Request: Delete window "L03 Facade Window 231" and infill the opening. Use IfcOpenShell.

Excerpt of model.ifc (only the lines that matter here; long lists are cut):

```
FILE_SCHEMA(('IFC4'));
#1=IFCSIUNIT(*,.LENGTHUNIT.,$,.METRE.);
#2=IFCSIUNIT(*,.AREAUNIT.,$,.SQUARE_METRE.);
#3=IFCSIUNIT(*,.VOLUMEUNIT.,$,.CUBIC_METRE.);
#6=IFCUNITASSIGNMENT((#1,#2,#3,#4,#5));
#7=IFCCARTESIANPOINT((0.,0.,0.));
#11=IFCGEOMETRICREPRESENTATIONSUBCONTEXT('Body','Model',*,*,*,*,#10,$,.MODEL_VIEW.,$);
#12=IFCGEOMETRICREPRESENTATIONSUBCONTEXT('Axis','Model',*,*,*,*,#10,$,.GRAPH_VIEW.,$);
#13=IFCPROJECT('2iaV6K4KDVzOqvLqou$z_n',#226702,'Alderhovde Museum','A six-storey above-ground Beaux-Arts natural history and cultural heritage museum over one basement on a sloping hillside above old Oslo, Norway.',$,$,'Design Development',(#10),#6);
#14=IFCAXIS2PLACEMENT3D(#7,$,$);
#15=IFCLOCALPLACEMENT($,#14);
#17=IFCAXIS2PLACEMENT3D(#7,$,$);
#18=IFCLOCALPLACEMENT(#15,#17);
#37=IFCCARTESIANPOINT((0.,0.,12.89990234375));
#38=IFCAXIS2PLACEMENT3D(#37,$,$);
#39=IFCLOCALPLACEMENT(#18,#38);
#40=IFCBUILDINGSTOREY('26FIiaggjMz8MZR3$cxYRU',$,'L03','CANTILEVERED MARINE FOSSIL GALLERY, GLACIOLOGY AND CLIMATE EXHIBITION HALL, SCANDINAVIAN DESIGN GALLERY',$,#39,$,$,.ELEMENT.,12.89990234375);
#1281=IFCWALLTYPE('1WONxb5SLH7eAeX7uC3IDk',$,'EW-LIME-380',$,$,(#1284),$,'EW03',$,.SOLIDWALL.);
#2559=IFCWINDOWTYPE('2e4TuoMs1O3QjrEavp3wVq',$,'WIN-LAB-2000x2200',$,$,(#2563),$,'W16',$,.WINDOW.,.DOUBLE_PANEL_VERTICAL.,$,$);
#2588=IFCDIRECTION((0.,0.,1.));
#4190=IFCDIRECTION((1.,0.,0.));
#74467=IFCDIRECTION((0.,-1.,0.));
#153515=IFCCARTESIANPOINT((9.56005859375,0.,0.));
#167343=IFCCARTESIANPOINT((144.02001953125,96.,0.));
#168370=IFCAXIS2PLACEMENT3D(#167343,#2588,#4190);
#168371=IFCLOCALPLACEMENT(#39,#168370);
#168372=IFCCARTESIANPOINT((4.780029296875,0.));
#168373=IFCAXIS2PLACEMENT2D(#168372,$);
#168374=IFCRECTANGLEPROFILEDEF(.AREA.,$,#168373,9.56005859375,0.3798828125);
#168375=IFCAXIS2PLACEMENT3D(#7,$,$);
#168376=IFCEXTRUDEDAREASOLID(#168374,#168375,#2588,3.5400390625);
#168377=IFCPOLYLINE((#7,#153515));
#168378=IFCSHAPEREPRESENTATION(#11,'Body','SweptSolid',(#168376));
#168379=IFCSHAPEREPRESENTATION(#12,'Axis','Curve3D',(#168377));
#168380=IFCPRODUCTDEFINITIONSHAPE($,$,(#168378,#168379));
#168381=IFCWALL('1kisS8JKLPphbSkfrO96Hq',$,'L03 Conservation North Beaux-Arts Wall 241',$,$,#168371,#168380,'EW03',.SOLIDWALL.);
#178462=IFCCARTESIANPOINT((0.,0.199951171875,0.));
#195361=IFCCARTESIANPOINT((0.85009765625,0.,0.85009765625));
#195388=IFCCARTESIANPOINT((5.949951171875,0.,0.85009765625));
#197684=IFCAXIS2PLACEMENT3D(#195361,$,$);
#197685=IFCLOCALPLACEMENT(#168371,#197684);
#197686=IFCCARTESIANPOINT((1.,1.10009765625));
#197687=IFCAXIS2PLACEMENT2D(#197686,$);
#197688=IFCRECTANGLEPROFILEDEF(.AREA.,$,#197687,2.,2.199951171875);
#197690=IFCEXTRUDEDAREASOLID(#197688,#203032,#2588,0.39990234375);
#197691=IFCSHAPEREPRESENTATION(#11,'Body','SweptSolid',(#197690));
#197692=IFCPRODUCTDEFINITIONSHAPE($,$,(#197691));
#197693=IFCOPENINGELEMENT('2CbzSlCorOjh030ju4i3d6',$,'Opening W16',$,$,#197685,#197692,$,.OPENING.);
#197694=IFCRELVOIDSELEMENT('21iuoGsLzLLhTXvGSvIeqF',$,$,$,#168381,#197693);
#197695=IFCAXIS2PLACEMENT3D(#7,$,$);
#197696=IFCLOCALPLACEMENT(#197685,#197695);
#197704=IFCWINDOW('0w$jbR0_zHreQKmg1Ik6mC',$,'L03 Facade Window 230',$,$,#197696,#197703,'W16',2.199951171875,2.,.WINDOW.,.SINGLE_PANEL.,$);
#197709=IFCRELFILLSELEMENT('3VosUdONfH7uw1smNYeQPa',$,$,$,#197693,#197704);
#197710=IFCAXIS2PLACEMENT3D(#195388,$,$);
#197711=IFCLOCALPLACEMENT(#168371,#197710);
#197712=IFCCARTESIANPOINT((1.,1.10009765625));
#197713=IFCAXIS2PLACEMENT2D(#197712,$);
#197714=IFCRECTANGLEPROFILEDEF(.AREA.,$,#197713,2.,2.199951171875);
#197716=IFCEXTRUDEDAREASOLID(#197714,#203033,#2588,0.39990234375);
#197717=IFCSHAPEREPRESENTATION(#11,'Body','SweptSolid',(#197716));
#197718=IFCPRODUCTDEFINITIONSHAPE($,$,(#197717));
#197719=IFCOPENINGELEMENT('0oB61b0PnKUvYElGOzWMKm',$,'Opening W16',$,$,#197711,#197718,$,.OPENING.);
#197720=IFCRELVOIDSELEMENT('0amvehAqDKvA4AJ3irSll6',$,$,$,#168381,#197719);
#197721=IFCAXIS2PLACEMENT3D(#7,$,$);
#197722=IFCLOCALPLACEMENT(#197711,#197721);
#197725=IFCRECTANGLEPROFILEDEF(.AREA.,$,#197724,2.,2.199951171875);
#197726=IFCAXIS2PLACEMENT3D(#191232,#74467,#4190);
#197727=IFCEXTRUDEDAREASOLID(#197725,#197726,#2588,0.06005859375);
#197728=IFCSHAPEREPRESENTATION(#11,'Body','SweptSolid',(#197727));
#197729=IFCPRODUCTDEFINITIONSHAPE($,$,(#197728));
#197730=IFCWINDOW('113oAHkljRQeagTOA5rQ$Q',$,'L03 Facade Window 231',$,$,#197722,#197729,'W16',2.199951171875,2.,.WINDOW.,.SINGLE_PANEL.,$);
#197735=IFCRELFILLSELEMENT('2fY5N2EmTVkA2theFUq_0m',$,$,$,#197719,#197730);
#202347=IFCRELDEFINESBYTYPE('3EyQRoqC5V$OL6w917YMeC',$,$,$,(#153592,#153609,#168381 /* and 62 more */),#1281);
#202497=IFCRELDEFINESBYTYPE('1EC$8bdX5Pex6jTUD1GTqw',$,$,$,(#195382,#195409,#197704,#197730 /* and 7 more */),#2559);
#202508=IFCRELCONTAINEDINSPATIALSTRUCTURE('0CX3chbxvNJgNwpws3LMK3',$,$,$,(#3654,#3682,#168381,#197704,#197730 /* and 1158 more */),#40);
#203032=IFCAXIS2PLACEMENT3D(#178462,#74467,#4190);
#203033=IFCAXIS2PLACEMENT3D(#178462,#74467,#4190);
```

```python
import ifcopenshell
import ifcopenshell.api.feature
import ifcopenshell.api.root
import ifcopenshell.geom
import ifcopenshell.util.shape

model = ifcopenshell.open("model.ifc")
settings = ifcopenshell.geom.settings()


def volume(element):
    """Net volume in cubic metres, openings subtracted."""
    shape = ifcopenshell.geom.create_shape(settings, element)
    return ifcopenshell.util.shape.get_volume(shape.geometry)


window = model.by_id(197730)
opening = window.FillsVoids[0].RelatingOpeningElement
wall = opening.VoidsElements[0].RelatingBuildingElement
before = volume(wall)

ifcopenshell.api.root.remove_product(model, product=window)
ifcopenshell.api.feature.remove_feature(model, feature=opening)

after = volume(wall)

print(f"wall volume {before:.3f} -> {after:.3f} m3")

model.write("model_rev.ifc")
```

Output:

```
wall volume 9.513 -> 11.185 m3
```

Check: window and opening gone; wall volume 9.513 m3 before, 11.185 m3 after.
